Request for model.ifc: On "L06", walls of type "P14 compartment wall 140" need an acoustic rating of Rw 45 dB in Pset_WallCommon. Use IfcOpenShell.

First a look at what the model holds.

```python
import ifcopenshell
import ifcopenshell.util.element

model = ifcopenshell.open("model.ifc")
print(model.schema)
storey = next(s for s in model.by_type("IfcBuildingStorey") if s.Name == "L06")
walls = [e for e in ifcopenshell.util.element.get_decomposition(storey) if e.is_a("IfcWall")]
seen = {}
for e in walls:
    element_type = ifcopenshell.util.element.get_type(e)
    key = (element_type.Name if element_type != e and element_type else None, ifcopenshell.util.element.get_pset(e, "Pset_WallCommon", "AcousticRating"))
    seen[key] = seen.get(key, 0) + 1
for (name, value), count in sorted(seen.items(), key=str):
    print(count, "x", name, "|", value)
```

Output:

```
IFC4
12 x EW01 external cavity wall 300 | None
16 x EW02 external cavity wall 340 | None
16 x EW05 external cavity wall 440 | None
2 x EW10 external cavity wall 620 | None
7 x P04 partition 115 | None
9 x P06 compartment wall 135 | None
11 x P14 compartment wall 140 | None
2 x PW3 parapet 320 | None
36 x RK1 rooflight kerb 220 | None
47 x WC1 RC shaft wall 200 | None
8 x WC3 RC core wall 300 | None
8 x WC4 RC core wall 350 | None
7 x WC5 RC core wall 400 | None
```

```python
import ifcopenshell
import ifcopenshell.api.pset
import ifcopenshell.util.element

model = ifcopenshell.open("model.ifc")

storey = next(s for s in model.by_type("IfcBuildingStorey") if s.Name == "L06")
walls = [e for e in ifcopenshell.util.element.get_decomposition(storey) if e.is_a("IfcWall")]

count = 0
for e in walls:
    element_type = ifcopenshell.util.element.get_type(e)
    if element_type in (None, e) or element_type.Name != "P14 compartment wall 140":
        continue
    # add_pset returns the element's existing set when there is one.
    pset = ifcopenshell.api.pset.add_pset(model, product=e, name="Pset_WallCommon")
    ifcopenshell.api.pset.edit_pset(model, pset=pset, properties={"AcousticRating": "Rw 45 dB"})
    count += 1

print(count, "walls updated")

model.write("model_updated.ifc")
```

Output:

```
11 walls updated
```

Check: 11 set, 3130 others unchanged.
